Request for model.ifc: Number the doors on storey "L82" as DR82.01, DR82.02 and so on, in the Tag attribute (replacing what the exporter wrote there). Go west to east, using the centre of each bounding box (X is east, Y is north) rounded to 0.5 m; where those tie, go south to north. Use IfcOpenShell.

First a look at what the model holds.

```python
import ifcopenshell
import ifcopenshell.util.element
import ifcopenshell.util.placement

model = ifcopenshell.open("model.ifc")
print(model.schema)
storey = next(s for s in model.by_type("IfcBuildingStorey") if s.Name == "L82")
doors = [e for e in ifcopenshell.util.element.get_decomposition(storey) if e.is_a("IfcDoor")]
for e in sorted(doors, key=lambda e: e.id()):
    origin = ifcopenshell.util.placement.get_local_placement(e.ObjectPlacement)[:3, 3]
    print(e.id(), e.Tag, e.Name, origin.round(2) + 0.0, sep=" | ")
```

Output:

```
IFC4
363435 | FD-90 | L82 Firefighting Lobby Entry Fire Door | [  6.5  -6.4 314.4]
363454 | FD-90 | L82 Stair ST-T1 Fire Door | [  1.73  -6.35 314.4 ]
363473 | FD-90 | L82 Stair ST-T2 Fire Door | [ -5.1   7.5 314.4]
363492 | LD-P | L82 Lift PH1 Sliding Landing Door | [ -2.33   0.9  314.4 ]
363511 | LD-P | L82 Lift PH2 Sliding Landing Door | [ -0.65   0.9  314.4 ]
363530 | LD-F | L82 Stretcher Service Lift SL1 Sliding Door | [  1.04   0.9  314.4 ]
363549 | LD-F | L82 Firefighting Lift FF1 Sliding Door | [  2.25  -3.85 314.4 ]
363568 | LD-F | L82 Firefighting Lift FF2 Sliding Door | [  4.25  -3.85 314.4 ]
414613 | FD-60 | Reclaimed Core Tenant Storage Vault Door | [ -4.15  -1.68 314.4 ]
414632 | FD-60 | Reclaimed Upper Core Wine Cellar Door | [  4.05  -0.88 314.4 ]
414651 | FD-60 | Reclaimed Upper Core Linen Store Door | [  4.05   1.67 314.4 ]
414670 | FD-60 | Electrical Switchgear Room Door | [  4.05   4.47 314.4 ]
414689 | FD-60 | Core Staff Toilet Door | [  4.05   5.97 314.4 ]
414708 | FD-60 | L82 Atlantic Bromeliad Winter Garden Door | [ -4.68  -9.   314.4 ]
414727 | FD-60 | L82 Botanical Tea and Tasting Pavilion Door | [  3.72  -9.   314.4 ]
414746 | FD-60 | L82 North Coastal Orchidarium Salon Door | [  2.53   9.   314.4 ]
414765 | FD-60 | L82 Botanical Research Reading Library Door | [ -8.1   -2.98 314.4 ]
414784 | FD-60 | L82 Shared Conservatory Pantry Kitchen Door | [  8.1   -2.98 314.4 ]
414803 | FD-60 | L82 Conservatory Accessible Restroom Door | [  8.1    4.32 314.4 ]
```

```python
import ifcopenshell
import ifcopenshell.geom
import ifcopenshell.util.element
import ifcopenshell.util.shape

model = ifcopenshell.open("model.ifc")
settings = ifcopenshell.geom.settings()
settings.set("use-world-coords", True)


def centre(element):
    shape = ifcopenshell.geom.create_shape(settings, element)
    return ifcopenshell.util.shape.get_bbox_centroid(shape.geometry)


storey = next(s for s in model.by_type("IfcBuildingStorey") if s.Name == "L82")
doors = [e for e in ifcopenshell.util.element.get_decomposition(storey) if e.is_a("IfcDoor")]

# Insertion points can sit at a corner or the storey origin, so sort by the geometry (in metres).
centres = {e: centre(e) for e in doors}
doors.sort(key=lambda e: (round(centres[e][0] / 0.5), centres[e][1]))

for i, e in enumerate(doors, start=1):
    number = f"DR82.{i:02d}"
    e.Tag = number
    print(e.id(), number)

model.write("model_edited.ifc")
```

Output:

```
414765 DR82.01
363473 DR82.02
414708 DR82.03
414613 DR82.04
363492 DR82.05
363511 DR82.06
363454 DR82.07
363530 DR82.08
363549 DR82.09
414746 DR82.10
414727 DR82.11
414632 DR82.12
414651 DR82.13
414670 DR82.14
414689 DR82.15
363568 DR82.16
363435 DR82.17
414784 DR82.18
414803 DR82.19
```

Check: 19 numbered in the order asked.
